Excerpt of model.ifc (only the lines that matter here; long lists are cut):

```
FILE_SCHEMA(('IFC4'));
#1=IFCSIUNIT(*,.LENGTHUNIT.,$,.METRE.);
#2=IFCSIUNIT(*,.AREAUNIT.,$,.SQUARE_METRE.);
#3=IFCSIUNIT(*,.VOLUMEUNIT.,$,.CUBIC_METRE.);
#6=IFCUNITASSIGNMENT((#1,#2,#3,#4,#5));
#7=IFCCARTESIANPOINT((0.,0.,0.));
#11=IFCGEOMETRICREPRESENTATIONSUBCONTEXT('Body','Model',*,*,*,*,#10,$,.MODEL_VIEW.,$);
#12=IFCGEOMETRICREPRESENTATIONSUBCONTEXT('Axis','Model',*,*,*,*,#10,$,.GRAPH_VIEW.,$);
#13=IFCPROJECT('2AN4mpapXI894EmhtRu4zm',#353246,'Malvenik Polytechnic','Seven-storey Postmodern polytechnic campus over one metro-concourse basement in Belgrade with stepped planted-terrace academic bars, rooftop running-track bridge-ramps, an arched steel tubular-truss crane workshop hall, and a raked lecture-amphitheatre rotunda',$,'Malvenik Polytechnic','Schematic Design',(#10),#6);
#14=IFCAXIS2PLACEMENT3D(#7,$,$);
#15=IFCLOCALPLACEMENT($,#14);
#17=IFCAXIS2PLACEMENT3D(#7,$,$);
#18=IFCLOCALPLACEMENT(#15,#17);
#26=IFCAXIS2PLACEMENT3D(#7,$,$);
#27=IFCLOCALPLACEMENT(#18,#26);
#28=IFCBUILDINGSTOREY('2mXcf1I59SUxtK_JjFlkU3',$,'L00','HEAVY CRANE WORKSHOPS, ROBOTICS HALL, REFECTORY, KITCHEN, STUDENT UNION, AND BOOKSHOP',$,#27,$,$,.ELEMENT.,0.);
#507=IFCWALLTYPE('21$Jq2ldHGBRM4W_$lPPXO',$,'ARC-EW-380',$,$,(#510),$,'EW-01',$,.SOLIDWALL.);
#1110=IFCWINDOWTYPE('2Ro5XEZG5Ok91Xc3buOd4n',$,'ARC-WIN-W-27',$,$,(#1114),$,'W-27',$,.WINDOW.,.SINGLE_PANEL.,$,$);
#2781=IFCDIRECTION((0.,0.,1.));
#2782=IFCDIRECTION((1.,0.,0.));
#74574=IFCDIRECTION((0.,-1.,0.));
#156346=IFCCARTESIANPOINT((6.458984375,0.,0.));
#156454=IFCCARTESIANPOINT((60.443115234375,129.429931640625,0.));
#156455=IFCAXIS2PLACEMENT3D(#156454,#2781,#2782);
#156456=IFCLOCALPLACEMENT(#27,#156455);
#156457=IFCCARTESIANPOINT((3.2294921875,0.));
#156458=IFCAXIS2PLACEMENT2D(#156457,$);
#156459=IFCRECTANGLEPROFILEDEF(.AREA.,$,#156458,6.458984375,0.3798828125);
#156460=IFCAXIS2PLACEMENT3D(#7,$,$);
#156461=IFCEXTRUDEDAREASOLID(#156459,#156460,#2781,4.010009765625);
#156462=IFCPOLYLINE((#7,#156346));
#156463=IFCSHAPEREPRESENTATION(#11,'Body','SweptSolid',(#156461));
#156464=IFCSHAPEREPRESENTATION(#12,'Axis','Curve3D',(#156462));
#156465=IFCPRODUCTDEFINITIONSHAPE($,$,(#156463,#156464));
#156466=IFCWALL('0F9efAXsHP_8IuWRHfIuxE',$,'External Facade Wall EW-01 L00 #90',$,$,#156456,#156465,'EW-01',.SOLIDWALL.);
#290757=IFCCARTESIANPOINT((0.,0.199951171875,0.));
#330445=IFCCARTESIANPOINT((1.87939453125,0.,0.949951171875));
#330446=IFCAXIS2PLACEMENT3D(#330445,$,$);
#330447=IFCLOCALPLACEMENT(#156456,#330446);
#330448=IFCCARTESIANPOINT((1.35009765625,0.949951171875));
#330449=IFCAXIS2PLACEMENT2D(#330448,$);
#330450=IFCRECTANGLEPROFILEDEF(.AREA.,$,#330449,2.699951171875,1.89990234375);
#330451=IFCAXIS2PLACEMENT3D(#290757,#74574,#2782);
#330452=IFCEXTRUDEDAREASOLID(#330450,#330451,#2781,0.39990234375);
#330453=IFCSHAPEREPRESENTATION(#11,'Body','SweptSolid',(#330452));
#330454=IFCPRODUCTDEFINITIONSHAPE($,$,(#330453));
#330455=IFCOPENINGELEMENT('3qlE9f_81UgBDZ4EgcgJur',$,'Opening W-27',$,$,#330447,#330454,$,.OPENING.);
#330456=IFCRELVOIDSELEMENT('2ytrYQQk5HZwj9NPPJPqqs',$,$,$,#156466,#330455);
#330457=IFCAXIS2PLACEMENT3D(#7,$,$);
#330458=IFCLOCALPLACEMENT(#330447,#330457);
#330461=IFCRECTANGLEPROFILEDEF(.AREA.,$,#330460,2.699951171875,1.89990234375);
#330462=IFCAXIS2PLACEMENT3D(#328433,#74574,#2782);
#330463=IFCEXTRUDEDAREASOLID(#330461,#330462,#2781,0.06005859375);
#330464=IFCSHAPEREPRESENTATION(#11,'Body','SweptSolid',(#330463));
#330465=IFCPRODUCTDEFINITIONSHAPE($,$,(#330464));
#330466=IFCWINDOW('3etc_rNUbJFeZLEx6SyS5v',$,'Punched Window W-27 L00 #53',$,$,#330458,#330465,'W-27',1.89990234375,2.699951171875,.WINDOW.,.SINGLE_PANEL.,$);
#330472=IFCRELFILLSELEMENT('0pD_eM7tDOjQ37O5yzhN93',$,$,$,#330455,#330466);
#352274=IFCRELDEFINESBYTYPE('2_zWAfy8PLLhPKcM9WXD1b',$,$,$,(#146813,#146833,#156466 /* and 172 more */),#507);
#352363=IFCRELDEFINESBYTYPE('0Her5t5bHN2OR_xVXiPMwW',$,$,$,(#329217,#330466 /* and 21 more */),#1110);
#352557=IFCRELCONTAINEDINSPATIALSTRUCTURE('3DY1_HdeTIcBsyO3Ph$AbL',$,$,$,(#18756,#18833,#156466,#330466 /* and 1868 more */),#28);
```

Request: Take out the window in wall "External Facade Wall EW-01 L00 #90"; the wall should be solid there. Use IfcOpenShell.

```python
import ifcopenshell
import ifcopenshell.api.feature
import ifcopenshell.api.root
import ifcopenshell.geom
import ifcopenshell.util.shape

model = ifcopenshell.open("model.ifc")
settings = ifcopenshell.geom.settings()


def volume(element):
    """Net volume in cubic metres, openings subtracted."""
    shape = ifcopenshell.geom.create_shape(settings, element)
    return ifcopenshell.util.shape.get_volume(shape.geometry)


window = model.by_guid("3etc_rNUbJFeZLEx6SyS5v")
opening = window.FillsVoids[0].RelatingOpeningElement
wall = opening.VoidsElements[0].RelatingBuildingElement
before = volume(wall)

ifcopenshell.api.root.remove_product(model, product=window)
ifcopenshell.api.feature.remove_feature(model, feature=opening)

after = volume(wall)

print(f"wall volume {before:.3f} -> {after:.3f} m3")

model.write("model_rev.ifc")
```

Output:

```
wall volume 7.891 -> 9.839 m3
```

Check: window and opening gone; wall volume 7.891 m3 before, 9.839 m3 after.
